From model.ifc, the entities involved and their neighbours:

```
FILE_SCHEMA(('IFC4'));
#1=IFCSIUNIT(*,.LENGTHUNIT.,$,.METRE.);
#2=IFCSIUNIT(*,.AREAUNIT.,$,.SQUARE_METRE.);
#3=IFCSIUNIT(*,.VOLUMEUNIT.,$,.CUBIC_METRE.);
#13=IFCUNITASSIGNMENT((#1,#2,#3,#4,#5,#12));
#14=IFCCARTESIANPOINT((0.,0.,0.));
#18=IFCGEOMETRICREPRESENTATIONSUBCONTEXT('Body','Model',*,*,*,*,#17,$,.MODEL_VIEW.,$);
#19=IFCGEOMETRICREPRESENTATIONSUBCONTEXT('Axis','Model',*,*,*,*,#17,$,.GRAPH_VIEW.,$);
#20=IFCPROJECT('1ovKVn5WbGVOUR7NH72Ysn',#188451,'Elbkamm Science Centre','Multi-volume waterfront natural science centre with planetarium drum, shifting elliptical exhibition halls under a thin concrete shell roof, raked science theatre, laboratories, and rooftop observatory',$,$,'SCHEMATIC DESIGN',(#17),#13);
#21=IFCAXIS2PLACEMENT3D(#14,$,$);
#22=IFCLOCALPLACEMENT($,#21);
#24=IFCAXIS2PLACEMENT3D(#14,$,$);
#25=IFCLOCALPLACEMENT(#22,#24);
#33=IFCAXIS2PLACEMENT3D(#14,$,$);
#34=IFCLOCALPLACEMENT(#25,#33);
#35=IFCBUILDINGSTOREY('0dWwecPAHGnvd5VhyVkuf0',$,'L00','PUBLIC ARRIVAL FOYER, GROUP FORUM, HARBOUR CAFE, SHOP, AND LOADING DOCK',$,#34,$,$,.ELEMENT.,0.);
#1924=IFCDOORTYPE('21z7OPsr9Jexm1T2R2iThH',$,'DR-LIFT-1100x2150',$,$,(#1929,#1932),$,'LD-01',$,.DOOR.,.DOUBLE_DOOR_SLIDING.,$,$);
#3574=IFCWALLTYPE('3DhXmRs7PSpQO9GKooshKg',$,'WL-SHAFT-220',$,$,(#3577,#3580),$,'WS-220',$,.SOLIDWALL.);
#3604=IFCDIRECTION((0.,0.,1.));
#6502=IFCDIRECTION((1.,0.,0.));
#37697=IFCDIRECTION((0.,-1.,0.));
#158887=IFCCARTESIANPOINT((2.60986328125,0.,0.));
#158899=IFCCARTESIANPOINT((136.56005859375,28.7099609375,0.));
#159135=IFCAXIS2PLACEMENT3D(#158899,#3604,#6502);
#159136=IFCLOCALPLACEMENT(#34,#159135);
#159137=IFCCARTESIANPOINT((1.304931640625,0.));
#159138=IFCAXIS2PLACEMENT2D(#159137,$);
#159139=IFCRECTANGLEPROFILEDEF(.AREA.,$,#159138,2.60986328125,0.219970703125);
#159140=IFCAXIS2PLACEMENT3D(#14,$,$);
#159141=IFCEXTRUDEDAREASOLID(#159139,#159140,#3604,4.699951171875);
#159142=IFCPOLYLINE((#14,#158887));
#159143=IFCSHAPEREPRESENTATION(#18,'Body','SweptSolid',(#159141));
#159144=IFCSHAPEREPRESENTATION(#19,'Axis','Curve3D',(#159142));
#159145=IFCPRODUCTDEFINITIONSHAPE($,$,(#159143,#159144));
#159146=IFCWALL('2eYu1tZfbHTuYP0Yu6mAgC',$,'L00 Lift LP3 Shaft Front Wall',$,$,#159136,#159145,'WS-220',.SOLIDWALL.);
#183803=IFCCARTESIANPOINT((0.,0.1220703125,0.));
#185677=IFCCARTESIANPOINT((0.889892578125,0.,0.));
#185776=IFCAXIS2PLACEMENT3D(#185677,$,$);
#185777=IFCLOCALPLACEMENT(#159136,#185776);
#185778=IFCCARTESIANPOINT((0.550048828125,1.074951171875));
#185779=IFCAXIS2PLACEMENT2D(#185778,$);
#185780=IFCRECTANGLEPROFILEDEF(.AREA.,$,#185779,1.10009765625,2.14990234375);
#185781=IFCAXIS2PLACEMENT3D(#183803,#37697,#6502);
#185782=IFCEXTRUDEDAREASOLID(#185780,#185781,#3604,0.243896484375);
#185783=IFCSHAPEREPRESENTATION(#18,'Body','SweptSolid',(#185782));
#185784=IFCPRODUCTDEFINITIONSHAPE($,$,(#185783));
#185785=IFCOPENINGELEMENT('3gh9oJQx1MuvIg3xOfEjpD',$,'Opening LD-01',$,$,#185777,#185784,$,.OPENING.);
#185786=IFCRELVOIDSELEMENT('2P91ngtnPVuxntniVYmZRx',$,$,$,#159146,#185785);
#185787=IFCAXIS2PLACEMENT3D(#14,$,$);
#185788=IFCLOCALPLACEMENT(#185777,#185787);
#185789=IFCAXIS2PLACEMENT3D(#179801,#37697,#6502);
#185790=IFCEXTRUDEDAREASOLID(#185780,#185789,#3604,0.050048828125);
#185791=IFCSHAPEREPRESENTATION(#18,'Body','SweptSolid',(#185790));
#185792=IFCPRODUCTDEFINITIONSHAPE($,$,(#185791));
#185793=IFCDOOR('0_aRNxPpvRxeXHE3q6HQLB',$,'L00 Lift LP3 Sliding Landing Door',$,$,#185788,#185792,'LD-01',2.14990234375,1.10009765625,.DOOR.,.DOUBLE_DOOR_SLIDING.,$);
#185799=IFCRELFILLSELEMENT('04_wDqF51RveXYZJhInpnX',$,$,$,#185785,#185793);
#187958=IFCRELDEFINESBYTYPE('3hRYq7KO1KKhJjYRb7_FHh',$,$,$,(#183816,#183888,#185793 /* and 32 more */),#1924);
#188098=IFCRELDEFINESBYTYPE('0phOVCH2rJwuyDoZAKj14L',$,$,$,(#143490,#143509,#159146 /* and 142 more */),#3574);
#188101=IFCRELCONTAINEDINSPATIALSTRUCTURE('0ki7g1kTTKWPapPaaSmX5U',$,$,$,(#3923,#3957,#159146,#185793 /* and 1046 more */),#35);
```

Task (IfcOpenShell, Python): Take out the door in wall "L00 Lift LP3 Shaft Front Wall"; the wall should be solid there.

```python
import ifcopenshell
import ifcopenshell.api.feature
import ifcopenshell.api.root
import ifcopenshell.geom
import ifcopenshell.util.shape

model = ifcopenshell.open("model.ifc")
settings = ifcopenshell.geom.settings()


def volume(element):
    """Net volume in cubic metres, openings subtracted."""
    shape = ifcopenshell.geom.create_shape(settings, element)
    return ifcopenshell.util.shape.get_volume(shape.geometry)


door = model.by_id(185793)
opening = door.FillsVoids[0].RelatingOpeningElement
wall = opening.VoidsElements[0].RelatingBuildingElement
before = volume(wall)

ifcopenshell.api.root.remove_product(model, product=door)
ifcopenshell.api.feature.remove_feature(model, feature=opening)

after = volume(wall)

print(f"wall volume {before:.3f} -> {after:.3f} m3")

model.write("model-out.ifc")
```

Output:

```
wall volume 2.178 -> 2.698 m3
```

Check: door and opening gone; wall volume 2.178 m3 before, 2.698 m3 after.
